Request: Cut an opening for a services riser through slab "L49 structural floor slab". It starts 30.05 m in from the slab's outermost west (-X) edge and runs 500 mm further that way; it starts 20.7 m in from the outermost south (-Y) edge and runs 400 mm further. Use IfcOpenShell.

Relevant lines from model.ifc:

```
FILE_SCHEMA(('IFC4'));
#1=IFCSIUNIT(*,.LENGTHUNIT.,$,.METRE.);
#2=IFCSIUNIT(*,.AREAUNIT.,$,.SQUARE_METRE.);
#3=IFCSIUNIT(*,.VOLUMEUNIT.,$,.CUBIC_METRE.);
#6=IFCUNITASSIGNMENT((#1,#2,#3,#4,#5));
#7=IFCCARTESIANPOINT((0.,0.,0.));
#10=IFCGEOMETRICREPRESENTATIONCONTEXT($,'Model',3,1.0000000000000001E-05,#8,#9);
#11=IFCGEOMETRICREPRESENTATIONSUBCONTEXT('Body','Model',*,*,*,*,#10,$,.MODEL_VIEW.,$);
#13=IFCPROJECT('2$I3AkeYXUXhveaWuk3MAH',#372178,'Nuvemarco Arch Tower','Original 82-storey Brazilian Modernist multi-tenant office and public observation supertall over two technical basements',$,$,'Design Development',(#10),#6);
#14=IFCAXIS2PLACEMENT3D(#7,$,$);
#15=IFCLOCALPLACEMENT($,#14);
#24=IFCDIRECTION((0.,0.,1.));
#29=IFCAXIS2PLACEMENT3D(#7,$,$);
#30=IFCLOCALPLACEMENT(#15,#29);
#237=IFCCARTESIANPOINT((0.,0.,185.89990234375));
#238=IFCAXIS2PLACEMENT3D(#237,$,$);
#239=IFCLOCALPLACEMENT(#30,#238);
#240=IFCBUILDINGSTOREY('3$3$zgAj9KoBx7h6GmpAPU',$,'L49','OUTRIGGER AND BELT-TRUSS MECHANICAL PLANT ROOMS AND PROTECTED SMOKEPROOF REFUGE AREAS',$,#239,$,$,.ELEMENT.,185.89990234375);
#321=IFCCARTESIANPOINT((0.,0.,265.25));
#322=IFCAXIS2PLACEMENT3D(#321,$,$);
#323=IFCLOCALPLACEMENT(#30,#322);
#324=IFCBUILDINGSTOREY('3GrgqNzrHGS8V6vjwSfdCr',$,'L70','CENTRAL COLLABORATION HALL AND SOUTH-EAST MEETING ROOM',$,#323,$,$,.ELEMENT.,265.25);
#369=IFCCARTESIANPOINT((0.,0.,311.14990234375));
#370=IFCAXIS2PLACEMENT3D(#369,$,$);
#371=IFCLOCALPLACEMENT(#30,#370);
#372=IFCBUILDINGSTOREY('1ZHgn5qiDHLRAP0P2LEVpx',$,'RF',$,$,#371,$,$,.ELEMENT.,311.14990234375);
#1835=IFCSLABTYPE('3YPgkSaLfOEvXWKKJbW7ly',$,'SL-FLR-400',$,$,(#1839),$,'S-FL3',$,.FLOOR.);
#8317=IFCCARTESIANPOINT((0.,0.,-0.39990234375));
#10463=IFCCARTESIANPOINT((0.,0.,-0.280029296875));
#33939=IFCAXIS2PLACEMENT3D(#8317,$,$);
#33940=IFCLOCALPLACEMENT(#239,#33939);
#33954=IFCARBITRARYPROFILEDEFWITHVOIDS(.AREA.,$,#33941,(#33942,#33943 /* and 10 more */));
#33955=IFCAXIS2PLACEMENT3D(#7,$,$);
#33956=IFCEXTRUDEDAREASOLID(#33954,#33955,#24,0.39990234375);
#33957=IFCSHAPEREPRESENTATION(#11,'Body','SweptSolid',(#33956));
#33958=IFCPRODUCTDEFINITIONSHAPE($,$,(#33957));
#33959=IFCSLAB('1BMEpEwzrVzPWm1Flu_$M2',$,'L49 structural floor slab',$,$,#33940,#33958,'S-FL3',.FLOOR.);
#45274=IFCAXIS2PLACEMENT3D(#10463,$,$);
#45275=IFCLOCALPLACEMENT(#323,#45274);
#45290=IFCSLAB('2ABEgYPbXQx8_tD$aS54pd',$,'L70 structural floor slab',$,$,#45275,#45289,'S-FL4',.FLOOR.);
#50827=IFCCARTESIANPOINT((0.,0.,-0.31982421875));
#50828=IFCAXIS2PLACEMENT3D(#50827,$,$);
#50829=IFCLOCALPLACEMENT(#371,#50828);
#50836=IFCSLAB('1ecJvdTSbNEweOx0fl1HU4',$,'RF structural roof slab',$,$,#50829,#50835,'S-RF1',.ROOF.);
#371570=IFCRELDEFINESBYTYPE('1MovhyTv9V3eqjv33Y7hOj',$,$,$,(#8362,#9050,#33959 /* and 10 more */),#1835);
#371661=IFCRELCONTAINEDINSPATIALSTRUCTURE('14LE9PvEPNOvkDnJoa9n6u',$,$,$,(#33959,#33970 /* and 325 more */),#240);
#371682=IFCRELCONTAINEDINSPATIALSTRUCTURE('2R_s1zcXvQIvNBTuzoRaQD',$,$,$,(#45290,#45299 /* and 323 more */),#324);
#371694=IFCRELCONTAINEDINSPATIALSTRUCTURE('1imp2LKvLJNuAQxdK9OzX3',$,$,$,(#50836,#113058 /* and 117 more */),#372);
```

```python
import numpy as np
import ifcopenshell
import ifcopenshell.api.feature
import ifcopenshell.api.geometry
import ifcopenshell.api.root
import ifcopenshell.geom
import ifcopenshell.util.placement
import ifcopenshell.util.representation
import ifcopenshell.util.shape
import ifcopenshell.util.unit

model = ifcopenshell.open("model.ifc")
unit_scale = ifcopenshell.util.unit.calculate_unit_scale(model)
settings = ifcopenshell.geom.settings()


def volume(element):
    """Net volume in cubic metres, openings subtracted."""
    shape = ifcopenshell.geom.create_shape(settings, element)
    return ifcopenshell.util.shape.get_volume(shape.geometry)


slab = model.by_guid("1BMEpEwzrVzPWm1Flu_$M2")
before = volume(slab)

# Extent in the slab's own axes, in metres. The edges named are its -X and -Y sides.
slab_shape = ifcopenshell.geom.create_shape(settings, slab)
vertices = ifcopenshell.util.shape.get_vertices(slab_shape.geometry)
x_min, y_min, bottom = vertices.min(axis=0)
top = vertices[:, 2].max()

opening = ifcopenshell.api.root.create_entity(model, ifc_class="IfcOpeningElement", name="Services riser opening", predefined_type="OPENING")
context = ifcopenshell.util.representation.get_context(model, "Model", "Body", "MODEL_VIEW")
width, depth = 0.5, 0.4
outline = [(0.0, 0.0), (width, 0.0), (width, depth), (0.0, depth), (0.0, 0.0)]
# Overshoot both faces by 50 mm so the cut is clean.
shape = ifcopenshell.api.geometry.add_slab_representation(
    model, context=context, depth=top - bottom + 0.1, polyline=outline
)
ifcopenshell.api.geometry.assign_representation(model, product=opening, representation=shape)

matrix = ifcopenshell.util.placement.get_local_placement(slab.ObjectPlacement)
matrix[:, 3] = matrix @ np.append(np.array([x_min + 30.05, y_min + 20.7, bottom - 0.05]) / unit_scale, 1.0)
ifcopenshell.api.geometry.edit_object_placement(model, product=opening, matrix=matrix, is_si=False)
ifcopenshell.api.feature.add_feature(model, feature=opening, element=slab)

after = volume(slab)

print(f"slab volume {before:.3f} -> {after:.3f} m3")

model.write("model_rev.ifc")
```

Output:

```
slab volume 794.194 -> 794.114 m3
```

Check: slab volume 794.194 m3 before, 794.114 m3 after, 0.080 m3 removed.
